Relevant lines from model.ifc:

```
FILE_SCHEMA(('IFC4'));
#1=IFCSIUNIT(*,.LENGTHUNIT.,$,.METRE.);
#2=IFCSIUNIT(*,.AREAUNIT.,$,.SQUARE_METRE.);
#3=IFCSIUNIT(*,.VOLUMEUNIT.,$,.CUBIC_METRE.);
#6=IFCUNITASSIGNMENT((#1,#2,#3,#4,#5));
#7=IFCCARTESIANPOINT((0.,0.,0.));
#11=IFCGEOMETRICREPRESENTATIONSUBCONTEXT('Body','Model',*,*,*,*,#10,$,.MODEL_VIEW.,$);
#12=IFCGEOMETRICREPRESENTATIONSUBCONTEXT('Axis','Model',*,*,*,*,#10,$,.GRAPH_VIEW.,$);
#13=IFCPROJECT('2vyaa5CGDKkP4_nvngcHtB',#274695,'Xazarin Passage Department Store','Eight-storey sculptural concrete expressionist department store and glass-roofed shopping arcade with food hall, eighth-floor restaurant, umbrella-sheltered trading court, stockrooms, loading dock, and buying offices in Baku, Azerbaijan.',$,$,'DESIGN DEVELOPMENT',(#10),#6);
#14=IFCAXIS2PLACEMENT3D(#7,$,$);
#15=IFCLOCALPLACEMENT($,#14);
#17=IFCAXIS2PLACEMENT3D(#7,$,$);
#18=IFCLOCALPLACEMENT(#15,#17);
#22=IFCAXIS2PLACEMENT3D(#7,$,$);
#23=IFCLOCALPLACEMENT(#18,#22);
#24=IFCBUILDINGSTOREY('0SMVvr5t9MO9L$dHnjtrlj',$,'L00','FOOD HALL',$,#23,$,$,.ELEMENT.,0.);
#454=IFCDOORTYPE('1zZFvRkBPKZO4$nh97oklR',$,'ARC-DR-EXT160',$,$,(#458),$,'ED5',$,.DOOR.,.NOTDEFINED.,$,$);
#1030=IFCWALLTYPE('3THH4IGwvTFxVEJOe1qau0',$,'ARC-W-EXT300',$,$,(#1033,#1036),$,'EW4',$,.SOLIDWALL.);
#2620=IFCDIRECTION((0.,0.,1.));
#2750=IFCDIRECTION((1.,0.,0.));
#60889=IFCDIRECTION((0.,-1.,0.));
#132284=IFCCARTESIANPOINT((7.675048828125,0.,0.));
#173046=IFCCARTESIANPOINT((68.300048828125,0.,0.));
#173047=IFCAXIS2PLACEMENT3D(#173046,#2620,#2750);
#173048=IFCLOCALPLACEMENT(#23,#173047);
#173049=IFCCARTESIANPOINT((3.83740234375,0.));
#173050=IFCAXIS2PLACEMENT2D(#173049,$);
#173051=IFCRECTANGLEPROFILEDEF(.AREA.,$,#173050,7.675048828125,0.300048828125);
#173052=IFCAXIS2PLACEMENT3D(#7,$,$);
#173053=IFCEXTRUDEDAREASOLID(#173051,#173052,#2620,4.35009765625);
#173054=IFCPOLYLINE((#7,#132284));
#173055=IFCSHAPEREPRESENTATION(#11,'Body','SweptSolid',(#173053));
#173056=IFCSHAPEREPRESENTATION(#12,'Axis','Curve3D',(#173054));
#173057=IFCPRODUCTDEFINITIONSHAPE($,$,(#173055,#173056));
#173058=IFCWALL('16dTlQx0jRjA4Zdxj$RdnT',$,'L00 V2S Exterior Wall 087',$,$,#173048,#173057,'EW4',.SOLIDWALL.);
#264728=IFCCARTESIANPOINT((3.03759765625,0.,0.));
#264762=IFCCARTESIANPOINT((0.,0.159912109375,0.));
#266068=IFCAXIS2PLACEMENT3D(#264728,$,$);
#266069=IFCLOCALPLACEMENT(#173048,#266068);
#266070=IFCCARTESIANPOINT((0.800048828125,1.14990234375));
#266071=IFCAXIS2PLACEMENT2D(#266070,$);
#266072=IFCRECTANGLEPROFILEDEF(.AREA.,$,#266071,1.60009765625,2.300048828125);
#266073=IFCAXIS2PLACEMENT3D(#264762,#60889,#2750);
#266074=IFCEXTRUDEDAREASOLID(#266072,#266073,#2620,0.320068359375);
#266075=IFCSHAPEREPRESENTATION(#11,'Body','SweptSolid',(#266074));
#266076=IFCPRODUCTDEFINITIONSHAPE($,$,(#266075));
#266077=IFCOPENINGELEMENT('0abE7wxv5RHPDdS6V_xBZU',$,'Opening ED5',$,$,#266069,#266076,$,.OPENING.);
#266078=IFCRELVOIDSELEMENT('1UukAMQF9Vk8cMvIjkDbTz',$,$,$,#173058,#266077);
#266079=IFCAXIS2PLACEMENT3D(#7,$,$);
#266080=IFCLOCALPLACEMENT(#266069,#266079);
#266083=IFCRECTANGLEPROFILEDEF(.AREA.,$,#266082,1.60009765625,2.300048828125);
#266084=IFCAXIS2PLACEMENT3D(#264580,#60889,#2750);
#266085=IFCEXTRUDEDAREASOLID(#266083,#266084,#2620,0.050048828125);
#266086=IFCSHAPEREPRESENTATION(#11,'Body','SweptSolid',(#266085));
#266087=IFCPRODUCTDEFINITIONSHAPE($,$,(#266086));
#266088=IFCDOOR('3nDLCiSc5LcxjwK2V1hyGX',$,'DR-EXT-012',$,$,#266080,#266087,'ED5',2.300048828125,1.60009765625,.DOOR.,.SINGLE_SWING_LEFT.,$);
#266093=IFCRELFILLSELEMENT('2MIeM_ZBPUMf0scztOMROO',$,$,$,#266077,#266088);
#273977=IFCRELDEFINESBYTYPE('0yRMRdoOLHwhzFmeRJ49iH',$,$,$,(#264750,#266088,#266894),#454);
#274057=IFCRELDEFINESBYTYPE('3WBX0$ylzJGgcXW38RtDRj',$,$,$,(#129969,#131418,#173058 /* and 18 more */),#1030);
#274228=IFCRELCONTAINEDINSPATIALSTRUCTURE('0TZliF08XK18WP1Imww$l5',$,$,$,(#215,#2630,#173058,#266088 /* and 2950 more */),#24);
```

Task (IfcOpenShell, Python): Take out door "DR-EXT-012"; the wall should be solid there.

```python
import ifcopenshell
import ifcopenshell.api.feature
import ifcopenshell.api.root
import ifcopenshell.geom
import ifcopenshell.util.shape

model = ifcopenshell.open("model.ifc")
settings = ifcopenshell.geom.settings()


def volume(element):
    """Net volume in cubic metres, openings subtracted."""
    shape = ifcopenshell.geom.create_shape(settings, element)
    return ifcopenshell.util.shape.get_volume(shape.geometry)


door = model.by_guid("3nDLCiSc5LcxjwK2V1hyGX")
opening = door.FillsVoids[0].RelatingOpeningElement
wall = opening.VoidsElements[0].RelatingBuildingElement
before = volume(wall)

ifcopenshell.api.root.remove_product(model, product=door)
ifcopenshell.api.feature.remove_feature(model, feature=opening)

after = volume(wall)

print(f"wall volume {before:.3f} -> {after:.3f} m3")

model.write("model-out.ifc")
```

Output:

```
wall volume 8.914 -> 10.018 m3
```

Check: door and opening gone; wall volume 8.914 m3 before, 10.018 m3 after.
